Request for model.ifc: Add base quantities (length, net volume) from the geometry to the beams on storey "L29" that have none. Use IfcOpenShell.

First a look at what the model holds.

```python
import ifcopenshell
import ifcopenshell.util.element
import ifcopenshell.util.unit

model = ifcopenshell.open("model.ifc")
print(model.schema)
for unit_type in ("LENGTHUNIT", "AREAUNIT", "VOLUMEUNIT"):
    print(unit_type, ifcopenshell.util.unit.calculate_unit_scale(model, unit_type))
storey = next(s for s in model.by_type("IfcBuildingStorey") if s.Name == "L29")
beams = [e for e in ifcopenshell.util.element.get_decomposition(storey) if e.is_a("IfcBeam")]
for e in sorted(beams, key=lambda e: e.id()):
    print(e.id(), e.is_a(), e.Name, list(ifcopenshell.util.element.get_psets(e, qtos_only=True)), sep=" | ")
```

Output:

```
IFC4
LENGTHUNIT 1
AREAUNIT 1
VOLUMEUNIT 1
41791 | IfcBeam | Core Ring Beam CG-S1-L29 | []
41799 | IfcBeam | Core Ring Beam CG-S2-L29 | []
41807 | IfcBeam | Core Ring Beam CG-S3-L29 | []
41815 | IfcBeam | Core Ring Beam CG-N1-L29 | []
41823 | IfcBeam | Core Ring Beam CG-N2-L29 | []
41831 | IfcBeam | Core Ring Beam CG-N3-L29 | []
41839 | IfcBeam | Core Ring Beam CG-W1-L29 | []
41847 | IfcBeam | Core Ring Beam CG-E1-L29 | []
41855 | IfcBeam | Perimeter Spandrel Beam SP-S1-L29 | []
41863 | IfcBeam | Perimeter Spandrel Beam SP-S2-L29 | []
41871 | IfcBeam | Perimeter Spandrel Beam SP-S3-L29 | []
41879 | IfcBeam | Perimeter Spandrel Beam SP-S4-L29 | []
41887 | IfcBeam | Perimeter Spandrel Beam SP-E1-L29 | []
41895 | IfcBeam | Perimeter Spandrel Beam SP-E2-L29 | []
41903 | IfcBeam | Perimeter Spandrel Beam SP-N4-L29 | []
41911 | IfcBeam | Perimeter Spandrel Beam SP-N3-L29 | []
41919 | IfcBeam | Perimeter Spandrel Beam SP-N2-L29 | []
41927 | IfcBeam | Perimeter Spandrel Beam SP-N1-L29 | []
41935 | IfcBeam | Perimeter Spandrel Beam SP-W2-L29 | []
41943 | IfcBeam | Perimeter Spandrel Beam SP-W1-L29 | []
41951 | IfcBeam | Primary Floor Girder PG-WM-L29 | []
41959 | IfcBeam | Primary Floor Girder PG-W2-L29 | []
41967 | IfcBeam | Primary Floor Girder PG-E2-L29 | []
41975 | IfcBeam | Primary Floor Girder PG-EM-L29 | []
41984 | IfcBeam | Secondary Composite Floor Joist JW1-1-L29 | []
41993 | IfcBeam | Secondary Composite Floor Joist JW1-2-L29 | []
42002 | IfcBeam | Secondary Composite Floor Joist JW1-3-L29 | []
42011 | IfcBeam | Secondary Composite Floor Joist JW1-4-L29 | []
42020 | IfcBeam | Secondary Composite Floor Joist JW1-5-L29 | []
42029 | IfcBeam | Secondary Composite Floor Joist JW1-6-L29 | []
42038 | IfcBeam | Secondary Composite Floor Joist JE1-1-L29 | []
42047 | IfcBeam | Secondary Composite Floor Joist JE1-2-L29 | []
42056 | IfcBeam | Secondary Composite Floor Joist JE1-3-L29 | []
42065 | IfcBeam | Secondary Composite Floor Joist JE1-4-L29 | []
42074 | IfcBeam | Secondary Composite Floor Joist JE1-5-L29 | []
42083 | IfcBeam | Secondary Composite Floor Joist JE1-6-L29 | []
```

```python
import ifcopenshell
import ifcopenshell.api.pset
import ifcopenshell.geom
import ifcopenshell.util.element
import ifcopenshell.util.shape
import ifcopenshell.util.unit

model = ifcopenshell.open("model.ifc")
unit_scale = ifcopenshell.util.unit.calculate_unit_scale(model)
volume_scale = ifcopenshell.util.unit.calculate_unit_scale(model, "VOLUMEUNIT")
settings = ifcopenshell.geom.settings()

storey = next(s for s in model.by_type("IfcBuildingStorey") if s.Name == "L29")
beams = [e for e in ifcopenshell.util.element.get_decomposition(storey) if e.is_a("IfcBeam")]

for e in sorted(beams, key=lambda e: e.id()):
    if ifcopenshell.util.element.get_psets(e, qtos_only=True, should_inherit=False):
        continue
    # Geometry comes back in metres, in the element's own axes.
    shape = ifcopenshell.geom.create_shape(settings, e)
    values = {
        "Length": ifcopenshell.util.shape.get_max_xyz(shape.geometry) / unit_scale,
        "NetVolume": ifcopenshell.util.shape.get_volume(shape.geometry) / volume_scale,
    }
    qto = ifcopenshell.api.pset.add_qto(model, product=e, name="Qto_BeamBaseQuantities")
    ifcopenshell.api.pset.edit_qto(model, qto=qto, properties=values)
    print(e.id(), {k: round(v, 3) for k, v in values.items()})

model.write("model_edited.ifc")
```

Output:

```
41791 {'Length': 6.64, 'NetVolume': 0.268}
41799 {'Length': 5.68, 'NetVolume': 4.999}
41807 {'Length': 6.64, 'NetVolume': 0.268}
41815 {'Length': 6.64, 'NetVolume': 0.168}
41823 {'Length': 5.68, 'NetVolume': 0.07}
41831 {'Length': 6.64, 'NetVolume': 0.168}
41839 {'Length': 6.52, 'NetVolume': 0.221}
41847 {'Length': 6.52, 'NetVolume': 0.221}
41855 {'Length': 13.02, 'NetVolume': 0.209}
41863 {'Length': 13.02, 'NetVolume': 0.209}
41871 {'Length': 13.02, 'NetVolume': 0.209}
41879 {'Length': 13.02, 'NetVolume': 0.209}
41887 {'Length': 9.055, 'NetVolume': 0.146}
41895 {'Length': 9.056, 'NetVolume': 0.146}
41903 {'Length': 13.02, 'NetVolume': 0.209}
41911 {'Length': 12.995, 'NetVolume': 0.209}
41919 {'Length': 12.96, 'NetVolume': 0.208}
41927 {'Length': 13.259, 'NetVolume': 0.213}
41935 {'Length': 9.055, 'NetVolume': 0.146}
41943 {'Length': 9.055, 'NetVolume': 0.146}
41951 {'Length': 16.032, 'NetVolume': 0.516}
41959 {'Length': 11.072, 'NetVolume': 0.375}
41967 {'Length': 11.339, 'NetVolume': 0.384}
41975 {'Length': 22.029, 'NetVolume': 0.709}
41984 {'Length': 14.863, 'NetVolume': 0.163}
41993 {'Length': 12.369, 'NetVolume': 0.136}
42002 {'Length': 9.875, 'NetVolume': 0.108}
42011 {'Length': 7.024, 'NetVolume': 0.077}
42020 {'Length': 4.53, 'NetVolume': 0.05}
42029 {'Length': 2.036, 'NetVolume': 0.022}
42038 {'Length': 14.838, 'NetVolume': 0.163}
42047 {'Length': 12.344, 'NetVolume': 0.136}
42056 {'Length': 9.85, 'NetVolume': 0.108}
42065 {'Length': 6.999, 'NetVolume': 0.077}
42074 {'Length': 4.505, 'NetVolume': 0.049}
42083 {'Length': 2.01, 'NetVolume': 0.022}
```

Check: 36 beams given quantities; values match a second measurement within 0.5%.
